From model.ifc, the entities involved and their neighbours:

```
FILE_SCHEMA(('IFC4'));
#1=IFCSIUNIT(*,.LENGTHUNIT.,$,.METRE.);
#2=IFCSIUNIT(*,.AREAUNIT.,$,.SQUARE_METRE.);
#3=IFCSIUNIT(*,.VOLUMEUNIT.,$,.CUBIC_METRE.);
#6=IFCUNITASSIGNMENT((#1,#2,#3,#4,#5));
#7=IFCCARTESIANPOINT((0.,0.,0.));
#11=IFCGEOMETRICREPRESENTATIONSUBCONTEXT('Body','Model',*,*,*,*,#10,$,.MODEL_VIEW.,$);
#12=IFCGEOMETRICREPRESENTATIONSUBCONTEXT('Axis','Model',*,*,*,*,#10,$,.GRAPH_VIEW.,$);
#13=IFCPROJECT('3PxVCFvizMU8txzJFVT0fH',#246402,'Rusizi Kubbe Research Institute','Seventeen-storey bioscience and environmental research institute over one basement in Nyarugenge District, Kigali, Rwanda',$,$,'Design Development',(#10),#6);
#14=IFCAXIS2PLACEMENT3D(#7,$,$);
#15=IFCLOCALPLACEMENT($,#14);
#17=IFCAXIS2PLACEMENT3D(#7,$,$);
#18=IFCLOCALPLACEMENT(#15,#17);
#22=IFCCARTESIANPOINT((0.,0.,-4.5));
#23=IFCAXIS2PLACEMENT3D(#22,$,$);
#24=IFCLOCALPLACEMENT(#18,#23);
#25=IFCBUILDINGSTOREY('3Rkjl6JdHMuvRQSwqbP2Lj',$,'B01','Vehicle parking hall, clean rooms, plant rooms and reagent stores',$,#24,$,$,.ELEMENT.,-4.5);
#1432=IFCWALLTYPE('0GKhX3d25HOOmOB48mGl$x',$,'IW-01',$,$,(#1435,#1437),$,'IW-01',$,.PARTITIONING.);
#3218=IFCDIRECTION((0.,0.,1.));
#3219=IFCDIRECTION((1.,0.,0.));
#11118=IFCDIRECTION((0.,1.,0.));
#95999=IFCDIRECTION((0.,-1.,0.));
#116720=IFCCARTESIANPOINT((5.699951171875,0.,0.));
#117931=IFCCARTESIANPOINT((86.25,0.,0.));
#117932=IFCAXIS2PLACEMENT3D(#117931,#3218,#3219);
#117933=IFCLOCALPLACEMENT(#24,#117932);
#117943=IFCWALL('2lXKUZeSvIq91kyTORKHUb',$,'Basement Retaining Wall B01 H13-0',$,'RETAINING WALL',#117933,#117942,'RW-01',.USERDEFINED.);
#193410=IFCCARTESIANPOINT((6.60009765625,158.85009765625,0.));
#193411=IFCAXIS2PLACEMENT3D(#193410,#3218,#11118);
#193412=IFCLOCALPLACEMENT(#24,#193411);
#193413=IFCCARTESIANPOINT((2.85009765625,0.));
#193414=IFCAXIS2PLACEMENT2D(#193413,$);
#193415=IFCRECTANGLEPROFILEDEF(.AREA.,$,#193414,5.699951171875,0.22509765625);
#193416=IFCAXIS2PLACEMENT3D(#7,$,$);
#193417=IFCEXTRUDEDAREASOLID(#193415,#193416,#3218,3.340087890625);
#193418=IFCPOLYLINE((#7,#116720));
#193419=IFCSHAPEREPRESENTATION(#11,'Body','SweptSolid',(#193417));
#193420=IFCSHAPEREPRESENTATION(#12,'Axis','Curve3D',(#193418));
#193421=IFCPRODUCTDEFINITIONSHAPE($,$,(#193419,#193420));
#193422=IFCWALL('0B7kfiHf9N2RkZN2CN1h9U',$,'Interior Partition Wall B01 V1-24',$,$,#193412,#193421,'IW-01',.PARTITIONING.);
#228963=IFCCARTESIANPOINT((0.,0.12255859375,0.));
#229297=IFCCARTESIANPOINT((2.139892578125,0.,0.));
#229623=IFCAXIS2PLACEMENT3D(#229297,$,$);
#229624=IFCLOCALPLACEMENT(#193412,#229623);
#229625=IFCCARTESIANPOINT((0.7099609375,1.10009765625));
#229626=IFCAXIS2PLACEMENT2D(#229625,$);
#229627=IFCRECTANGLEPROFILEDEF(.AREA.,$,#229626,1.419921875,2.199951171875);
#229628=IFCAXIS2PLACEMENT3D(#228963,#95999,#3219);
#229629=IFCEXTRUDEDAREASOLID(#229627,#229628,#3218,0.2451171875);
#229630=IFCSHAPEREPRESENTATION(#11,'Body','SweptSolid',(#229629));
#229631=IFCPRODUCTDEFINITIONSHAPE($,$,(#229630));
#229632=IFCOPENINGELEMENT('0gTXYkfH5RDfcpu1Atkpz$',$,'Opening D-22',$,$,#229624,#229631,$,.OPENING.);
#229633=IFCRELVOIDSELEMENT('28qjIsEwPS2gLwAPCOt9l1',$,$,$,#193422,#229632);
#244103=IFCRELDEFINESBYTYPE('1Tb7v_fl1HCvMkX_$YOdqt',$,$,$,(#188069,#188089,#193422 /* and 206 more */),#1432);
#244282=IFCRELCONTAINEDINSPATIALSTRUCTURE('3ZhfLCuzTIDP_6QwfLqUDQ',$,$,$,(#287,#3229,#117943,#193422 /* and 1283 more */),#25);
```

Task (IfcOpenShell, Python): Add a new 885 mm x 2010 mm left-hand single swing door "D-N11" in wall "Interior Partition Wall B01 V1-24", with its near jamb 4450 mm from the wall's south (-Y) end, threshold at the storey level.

```python
import numpy as np
import ifcopenshell
import ifcopenshell.api.feature
import ifcopenshell.api.geometry
import ifcopenshell.api.root
import ifcopenshell.api.spatial
import ifcopenshell.geom
import ifcopenshell.util.element
import ifcopenshell.util.placement
import ifcopenshell.util.representation
import ifcopenshell.util.shape
import ifcopenshell.util.unit

model = ifcopenshell.open("model.ifc")
unit_scale = ifcopenshell.util.unit.calculate_unit_scale(model)
settings = ifcopenshell.geom.settings()


def volume(element):
    """Net volume in cubic metres, openings subtracted."""
    shape = ifcopenshell.geom.create_shape(settings, element)
    return ifcopenshell.util.shape.get_volume(shape.geometry)


wall = model.by_guid("0B7kfiHf9N2RkZN2CN1h9U")
storey = ifcopenshell.util.element.get_container(wall, ifc_class="IfcBuildingStorey")
context = ifcopenshell.util.representation.get_context(model, "Model", "Body", "MODEL_VIEW")
before = volume(wall)

width, height, from_end, sill = 0.885, 2.01, 4.45, 0.0  # metres

# The wall runs along its own X axis, and the end named is its -X end.
wall_shape = ifcopenshell.geom.create_shape(settings, wall)
x, y, z = ifcopenshell.util.shape.get_vertices(wall_shape.geometry).T
start = x.min() + from_end
face, thickness = float(y.min()), float(y.max() - y.min())
wall_matrix = ifcopenshell.util.placement.get_local_placement(wall.ObjectPlacement)
level = ifcopenshell.util.placement.get_local_placement(storey.ObjectPlacement)[2, 3]


def in_wall(x, y):
    """Placement at x, y metres in the wall's axes, at sill height."""
    matrix = wall_matrix.copy()
    matrix[:, 3] = wall_matrix @ np.array([x / unit_scale, y / unit_scale, 0.0, 1.0])
    matrix[2, 3] = level + sill / unit_scale
    return matrix


# Opening: a box that overshoots both wall faces by 50 mm.
opening = ifcopenshell.api.root.create_entity(model, ifc_class="IfcOpeningElement", predefined_type="OPENING")
box = ifcopenshell.api.geometry.add_wall_representation(
    model, context=context, length=width, height=height, thickness=thickness + 0.1
)
ifcopenshell.api.geometry.assign_representation(model, product=opening, representation=box)
ifcopenshell.api.geometry.edit_object_placement(model, product=opening, matrix=in_wall(start, face - 0.05), is_si=False)
ifcopenshell.api.feature.add_feature(model, feature=opening, element=wall)

door = ifcopenshell.api.root.create_entity(model, ifc_class="IfcDoor", name="D-N11", predefined_type="DOOR")
door.OverallWidth, door.OverallHeight = width / unit_scale, height / unit_scale
door.OperationType = "SINGLE_SWING_LEFT"
body = ifcopenshell.api.geometry.add_door_representation(
    model,
    context=context,
    overall_width=door.OverallWidth,
    overall_height=door.OverallHeight,
    operation_type="SINGLE_SWING_LEFT",
    lining_properties={"LiningDepth": thickness / unit_scale, "ThresholdDepth": thickness / unit_scale},
)
ifcopenshell.api.geometry.assign_representation(model, product=door, representation=body)
ifcopenshell.api.spatial.assign_container(model, products=[door], relating_structure=storey)
ifcopenshell.api.feature.add_filling(model, opening=opening, element=door)

# The lining spans the wall, so the door starts at the wall face.
ifcopenshell.api.geometry.edit_object_placement(model, product=door, matrix=in_wall(start, face), is_si=False)

after = volume(wall)

print(f"wall volume {before:.3f} -> {after:.3f} m3")

model.write("model_updated.ifc")
```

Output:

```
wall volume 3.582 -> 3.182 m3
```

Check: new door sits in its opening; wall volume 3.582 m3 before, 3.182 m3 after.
